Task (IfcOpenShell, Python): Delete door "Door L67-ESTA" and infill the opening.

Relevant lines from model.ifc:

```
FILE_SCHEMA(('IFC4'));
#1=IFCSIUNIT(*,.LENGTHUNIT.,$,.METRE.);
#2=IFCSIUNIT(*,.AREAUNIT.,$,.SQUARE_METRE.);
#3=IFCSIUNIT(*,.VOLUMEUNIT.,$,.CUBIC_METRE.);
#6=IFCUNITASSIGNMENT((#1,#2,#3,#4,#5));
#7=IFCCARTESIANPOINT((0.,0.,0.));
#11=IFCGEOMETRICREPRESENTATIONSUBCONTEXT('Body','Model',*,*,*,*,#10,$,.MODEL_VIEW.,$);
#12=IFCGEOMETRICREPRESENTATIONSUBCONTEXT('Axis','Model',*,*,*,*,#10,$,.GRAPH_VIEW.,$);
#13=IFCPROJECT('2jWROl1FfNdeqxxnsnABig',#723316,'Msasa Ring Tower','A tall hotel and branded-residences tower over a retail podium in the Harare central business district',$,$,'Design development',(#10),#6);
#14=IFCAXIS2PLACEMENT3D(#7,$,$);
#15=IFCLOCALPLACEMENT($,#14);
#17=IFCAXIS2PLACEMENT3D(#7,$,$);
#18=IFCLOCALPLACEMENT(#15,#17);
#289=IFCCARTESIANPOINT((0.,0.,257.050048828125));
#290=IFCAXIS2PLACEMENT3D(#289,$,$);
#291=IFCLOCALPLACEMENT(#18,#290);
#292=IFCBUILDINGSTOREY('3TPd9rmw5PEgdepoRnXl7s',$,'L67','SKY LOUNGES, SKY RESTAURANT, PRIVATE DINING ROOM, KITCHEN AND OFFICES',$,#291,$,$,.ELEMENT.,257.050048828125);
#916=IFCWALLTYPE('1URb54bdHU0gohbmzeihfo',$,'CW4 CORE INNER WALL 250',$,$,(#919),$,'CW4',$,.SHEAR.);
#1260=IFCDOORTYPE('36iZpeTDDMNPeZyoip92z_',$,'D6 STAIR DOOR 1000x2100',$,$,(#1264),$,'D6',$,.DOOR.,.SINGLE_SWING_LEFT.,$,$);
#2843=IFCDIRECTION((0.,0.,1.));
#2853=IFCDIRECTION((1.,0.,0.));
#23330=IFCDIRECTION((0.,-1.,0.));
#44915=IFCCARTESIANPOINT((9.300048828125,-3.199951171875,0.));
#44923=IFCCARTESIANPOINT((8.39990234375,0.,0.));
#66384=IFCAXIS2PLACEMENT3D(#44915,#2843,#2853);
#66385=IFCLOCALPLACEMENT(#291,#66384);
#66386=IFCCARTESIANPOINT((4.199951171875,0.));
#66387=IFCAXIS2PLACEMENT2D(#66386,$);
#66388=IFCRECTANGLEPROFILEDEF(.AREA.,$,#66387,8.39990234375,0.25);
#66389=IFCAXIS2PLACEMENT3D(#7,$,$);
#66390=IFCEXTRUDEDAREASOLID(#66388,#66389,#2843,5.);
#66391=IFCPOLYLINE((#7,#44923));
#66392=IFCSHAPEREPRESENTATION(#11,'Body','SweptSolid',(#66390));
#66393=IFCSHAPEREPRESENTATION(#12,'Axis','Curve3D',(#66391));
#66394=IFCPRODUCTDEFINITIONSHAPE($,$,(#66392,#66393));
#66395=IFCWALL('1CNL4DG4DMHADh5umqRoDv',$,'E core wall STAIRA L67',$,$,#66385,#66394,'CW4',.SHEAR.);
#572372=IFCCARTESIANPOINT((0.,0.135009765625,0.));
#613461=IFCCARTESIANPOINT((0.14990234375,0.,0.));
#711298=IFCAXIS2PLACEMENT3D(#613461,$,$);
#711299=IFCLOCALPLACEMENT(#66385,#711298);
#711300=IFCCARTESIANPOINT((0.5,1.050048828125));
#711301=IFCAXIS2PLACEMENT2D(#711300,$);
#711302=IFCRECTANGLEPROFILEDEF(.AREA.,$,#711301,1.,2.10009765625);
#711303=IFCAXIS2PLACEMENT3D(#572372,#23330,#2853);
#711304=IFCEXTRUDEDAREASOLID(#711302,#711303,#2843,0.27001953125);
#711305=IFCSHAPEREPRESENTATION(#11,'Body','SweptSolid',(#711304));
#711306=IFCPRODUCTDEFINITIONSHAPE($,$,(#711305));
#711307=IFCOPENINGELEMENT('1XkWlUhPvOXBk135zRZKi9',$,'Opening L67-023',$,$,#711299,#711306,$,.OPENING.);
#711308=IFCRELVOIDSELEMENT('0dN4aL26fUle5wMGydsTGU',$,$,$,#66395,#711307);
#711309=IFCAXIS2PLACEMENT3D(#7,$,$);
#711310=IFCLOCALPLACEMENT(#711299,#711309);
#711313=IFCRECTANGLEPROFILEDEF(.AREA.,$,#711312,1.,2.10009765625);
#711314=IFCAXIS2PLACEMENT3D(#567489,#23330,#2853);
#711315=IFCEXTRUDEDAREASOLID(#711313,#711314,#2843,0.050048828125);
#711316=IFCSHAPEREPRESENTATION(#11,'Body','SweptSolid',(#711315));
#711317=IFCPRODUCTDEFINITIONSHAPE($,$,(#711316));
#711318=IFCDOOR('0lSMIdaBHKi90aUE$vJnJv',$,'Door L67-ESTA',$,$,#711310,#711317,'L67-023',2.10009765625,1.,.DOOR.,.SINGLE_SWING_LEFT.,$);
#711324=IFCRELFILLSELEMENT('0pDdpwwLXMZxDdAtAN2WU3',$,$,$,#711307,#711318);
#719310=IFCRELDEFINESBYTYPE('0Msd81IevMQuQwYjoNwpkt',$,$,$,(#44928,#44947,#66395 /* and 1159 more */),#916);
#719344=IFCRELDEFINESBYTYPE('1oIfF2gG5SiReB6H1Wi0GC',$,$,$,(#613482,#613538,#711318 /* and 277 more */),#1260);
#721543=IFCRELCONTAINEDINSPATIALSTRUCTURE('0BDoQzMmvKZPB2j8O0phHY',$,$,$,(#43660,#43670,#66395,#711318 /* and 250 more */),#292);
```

```python
import ifcopenshell
import ifcopenshell.api.feature
import ifcopenshell.api.root
import ifcopenshell.geom
import ifcopenshell.util.shape

model = ifcopenshell.open("model.ifc")
settings = ifcopenshell.geom.settings()


def volume(element):
    """Net volume in cubic metres, openings subtracted."""
    shape = ifcopenshell.geom.create_shape(settings, element)
    return ifcopenshell.util.shape.get_volume(shape.geometry)


door = model.by_guid("0lSMIdaBHKi90aUE$vJnJv")
opening = door.FillsVoids[0].RelatingOpeningElement
wall = opening.VoidsElements[0].RelatingBuildingElement
before = volume(wall)

ifcopenshell.api.root.remove_product(model, product=door)
ifcopenshell.api.feature.remove_feature(model, feature=opening)

after = volume(wall)

print(f"wall volume {before:.3f} -> {after:.3f} m3")

model.write("model_rev.ifc")
```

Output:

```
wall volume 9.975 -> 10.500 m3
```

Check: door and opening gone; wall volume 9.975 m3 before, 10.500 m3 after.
